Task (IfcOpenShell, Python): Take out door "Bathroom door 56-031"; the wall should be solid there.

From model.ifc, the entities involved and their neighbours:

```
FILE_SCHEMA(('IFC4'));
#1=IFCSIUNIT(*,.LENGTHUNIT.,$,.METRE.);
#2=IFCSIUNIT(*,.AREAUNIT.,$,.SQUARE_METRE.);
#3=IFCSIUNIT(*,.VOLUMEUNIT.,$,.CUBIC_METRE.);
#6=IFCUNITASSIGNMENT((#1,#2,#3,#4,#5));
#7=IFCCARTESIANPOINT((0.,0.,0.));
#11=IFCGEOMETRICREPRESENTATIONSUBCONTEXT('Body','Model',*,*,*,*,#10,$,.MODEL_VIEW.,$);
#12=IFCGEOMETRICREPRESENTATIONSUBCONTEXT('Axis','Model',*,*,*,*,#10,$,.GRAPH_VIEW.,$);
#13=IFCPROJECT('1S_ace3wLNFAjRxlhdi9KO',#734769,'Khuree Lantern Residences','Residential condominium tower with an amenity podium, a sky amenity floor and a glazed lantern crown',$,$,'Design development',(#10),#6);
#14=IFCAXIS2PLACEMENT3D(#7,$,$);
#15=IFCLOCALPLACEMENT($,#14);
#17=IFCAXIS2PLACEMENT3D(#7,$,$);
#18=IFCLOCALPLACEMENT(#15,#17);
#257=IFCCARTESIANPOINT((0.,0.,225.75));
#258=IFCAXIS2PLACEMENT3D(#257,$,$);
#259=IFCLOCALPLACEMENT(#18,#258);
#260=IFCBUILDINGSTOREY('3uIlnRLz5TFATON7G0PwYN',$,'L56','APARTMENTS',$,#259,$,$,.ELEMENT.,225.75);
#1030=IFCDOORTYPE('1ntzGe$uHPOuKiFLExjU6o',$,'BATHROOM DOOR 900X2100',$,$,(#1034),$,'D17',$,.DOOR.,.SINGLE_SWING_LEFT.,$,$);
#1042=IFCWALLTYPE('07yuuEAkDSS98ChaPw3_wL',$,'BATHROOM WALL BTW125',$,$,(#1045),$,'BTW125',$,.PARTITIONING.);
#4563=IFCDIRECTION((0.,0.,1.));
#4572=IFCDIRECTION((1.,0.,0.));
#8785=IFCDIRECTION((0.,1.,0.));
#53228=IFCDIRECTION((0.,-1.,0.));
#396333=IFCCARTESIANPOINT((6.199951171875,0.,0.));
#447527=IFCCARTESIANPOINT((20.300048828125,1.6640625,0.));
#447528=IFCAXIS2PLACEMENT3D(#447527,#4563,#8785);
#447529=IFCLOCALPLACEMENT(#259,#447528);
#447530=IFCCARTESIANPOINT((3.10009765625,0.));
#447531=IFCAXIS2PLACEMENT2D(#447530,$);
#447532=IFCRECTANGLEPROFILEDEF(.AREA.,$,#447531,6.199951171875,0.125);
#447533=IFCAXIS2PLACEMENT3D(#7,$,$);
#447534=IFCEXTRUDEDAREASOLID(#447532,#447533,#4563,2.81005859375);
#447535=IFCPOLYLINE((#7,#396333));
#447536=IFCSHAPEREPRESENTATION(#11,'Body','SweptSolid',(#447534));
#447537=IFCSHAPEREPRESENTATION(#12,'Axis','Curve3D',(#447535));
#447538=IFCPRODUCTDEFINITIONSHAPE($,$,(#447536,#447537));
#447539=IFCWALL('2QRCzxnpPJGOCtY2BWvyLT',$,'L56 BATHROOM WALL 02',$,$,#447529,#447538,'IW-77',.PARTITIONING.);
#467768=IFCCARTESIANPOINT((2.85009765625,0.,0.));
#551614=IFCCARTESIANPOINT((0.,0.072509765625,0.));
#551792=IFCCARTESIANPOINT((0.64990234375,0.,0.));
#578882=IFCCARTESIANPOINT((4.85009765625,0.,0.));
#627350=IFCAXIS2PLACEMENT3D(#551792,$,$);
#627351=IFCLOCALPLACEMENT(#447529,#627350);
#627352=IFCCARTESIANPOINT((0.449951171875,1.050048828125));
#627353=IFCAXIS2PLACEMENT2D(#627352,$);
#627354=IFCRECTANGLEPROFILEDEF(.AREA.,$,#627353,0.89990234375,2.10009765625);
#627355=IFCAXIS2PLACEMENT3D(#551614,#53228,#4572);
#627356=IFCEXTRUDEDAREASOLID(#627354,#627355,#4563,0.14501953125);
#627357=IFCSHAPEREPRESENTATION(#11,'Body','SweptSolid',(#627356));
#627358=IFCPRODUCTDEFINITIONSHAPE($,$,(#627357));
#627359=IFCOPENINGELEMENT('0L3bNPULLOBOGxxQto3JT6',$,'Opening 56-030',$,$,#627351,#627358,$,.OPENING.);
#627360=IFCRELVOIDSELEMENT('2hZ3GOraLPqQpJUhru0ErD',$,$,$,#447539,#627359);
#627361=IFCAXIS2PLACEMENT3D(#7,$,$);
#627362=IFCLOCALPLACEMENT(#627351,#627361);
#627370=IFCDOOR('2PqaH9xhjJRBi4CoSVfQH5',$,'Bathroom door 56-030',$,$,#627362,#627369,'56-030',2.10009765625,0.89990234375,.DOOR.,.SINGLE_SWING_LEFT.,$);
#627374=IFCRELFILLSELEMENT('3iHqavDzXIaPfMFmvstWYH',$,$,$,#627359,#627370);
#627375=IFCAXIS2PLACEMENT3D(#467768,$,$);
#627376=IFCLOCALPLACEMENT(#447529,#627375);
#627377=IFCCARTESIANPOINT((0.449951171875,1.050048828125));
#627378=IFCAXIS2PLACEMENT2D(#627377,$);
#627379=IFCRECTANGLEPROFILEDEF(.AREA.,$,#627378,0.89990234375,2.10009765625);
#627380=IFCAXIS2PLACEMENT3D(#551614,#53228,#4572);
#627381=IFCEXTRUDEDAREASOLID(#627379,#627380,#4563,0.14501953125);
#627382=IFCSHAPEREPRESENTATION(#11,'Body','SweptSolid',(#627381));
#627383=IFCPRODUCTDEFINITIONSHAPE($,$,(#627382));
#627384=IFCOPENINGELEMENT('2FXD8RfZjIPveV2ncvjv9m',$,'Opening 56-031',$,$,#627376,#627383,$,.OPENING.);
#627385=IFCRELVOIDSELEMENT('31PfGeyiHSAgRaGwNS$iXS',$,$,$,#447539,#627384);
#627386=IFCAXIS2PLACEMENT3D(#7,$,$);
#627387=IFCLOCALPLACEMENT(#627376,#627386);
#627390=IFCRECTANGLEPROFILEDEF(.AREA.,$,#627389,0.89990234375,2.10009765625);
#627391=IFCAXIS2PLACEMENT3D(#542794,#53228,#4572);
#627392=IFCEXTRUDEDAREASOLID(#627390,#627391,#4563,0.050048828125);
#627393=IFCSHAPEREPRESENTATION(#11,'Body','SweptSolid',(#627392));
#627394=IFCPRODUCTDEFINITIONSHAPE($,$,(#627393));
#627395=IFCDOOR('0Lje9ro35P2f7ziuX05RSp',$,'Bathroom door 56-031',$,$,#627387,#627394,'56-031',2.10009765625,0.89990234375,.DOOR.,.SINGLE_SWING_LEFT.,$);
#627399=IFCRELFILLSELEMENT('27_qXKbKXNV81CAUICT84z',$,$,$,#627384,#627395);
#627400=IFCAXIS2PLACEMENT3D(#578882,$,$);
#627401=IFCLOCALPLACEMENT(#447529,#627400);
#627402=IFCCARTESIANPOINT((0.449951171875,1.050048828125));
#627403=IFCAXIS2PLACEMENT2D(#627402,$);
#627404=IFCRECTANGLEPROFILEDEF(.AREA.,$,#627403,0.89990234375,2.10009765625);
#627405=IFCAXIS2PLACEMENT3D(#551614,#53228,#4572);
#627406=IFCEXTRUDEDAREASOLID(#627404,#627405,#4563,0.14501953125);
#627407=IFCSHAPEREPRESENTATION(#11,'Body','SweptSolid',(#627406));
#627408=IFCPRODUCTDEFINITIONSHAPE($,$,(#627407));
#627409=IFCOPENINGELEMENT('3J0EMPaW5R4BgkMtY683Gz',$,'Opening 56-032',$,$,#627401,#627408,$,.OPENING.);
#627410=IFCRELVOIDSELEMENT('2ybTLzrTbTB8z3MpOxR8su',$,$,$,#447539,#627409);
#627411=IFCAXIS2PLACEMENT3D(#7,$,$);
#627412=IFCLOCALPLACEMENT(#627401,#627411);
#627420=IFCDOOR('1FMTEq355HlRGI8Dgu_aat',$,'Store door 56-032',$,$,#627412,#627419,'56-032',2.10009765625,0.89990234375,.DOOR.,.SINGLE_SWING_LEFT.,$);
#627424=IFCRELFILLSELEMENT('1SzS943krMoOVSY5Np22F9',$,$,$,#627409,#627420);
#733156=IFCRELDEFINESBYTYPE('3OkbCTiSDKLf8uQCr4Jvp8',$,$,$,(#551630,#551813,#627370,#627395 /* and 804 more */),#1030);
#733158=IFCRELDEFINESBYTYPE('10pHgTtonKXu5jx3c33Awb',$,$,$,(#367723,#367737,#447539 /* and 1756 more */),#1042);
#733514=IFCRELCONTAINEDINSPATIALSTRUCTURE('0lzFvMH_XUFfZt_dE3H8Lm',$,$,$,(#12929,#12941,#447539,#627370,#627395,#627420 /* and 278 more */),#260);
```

```python
import ifcopenshell
import ifcopenshell.api.feature
import ifcopenshell.api.root
import ifcopenshell.geom
import ifcopenshell.util.shape

model = ifcopenshell.open("model.ifc")
settings = ifcopenshell.geom.settings()


def volume(element):
    """Net volume in cubic metres, openings subtracted."""
    shape = ifcopenshell.geom.create_shape(settings, element)
    return ifcopenshell.util.shape.get_volume(shape.geometry)


door = model.by_id(627395)
opening = door.FillsVoids[0].RelatingOpeningElement
wall = opening.VoidsElements[0].RelatingBuildingElement
before = volume(wall)

ifcopenshell.api.root.remove_product(model, product=door)
ifcopenshell.api.feature.remove_feature(model, feature=opening)

after = volume(wall)

print(f"wall volume {before:.3f} -> {after:.3f} m3")

model.write("model_rev.ifc")
```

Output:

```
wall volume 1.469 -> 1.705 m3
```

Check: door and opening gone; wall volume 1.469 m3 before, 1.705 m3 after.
